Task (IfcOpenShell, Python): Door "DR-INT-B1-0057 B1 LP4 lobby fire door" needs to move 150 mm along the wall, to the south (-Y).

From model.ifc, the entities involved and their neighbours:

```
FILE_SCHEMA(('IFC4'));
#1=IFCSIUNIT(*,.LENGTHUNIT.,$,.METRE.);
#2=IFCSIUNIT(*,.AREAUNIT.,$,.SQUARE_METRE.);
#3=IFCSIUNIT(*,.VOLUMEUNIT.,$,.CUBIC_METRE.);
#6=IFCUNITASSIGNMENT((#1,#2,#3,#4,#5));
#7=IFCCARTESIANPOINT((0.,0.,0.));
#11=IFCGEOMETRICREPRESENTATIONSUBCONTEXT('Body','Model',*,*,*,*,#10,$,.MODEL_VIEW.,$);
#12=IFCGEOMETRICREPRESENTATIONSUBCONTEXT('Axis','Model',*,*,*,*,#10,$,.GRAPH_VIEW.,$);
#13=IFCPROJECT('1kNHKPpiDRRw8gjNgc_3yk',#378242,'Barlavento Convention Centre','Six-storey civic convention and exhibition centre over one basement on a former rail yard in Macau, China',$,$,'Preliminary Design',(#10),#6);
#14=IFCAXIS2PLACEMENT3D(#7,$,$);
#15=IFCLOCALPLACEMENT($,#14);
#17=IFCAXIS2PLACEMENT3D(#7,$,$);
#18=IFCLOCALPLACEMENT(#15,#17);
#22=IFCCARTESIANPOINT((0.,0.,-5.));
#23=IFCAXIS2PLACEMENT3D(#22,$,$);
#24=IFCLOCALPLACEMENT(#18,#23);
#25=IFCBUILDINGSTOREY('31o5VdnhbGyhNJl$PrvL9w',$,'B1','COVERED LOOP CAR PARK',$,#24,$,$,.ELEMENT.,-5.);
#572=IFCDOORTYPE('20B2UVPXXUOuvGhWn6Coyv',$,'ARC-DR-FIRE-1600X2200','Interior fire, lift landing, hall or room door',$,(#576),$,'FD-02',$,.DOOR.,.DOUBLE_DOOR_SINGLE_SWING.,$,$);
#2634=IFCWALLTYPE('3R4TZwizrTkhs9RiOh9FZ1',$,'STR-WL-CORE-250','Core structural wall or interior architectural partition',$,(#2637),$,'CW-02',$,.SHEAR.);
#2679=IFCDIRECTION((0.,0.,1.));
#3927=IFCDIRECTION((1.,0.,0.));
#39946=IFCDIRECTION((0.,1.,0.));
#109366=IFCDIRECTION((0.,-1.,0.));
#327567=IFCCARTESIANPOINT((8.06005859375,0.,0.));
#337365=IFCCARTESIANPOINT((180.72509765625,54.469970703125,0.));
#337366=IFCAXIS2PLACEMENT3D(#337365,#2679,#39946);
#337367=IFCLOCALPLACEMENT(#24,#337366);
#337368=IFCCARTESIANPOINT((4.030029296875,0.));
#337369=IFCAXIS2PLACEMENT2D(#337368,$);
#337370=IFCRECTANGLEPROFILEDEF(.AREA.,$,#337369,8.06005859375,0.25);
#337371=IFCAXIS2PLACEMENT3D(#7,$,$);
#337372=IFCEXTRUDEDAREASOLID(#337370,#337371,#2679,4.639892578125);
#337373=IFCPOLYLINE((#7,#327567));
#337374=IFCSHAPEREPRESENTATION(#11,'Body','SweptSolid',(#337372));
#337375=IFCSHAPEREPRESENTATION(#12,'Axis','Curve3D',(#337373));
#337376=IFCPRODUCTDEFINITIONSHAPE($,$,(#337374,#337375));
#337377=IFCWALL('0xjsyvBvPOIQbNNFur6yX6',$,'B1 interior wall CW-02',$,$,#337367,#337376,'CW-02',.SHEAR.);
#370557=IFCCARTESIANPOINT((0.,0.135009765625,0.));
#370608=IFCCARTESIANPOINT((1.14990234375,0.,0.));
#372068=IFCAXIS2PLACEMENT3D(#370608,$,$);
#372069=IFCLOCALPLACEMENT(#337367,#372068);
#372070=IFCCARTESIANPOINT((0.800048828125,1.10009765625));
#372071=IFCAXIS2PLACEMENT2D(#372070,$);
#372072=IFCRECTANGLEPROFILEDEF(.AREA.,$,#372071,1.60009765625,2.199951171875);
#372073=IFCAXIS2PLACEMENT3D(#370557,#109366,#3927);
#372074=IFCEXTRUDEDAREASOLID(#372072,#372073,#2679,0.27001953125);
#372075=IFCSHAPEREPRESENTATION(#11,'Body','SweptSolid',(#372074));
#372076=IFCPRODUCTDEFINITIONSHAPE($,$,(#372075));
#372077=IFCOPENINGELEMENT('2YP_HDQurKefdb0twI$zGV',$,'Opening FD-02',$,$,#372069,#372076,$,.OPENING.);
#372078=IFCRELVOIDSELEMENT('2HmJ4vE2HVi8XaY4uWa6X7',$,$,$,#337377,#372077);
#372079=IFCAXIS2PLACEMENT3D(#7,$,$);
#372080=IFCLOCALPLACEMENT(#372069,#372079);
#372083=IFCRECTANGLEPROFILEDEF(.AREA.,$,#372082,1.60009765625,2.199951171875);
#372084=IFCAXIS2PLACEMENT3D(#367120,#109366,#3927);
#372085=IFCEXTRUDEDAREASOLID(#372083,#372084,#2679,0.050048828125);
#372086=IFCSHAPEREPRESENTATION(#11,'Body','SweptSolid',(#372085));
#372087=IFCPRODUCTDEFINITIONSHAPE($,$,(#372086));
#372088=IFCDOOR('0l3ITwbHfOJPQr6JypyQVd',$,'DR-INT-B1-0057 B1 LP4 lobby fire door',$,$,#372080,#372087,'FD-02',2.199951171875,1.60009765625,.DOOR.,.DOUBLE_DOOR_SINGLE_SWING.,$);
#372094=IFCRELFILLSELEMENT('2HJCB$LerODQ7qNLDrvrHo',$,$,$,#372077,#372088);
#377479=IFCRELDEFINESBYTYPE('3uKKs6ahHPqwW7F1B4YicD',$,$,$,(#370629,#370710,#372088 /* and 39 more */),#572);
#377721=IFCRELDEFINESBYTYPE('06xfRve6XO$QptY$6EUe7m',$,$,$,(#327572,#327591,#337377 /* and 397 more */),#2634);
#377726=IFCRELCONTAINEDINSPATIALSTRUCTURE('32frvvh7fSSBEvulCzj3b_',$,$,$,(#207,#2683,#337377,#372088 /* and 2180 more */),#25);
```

```python
import ifcopenshell
import ifcopenshell.api.geometry
import ifcopenshell.util.placement

model = ifcopenshell.open("model.ifc")

door = model.by_guid("0l3ITwbHfOJPQr6JypyQVd")
opening = door.FillsVoids[0].RelatingOpeningElement
wall = opening.VoidsElements[0].RelatingBuildingElement

wall_matrix = ifcopenshell.util.placement.get_local_placement(wall.ObjectPlacement)
shift = wall_matrix[:3, 0] * -0.15
before = ifcopenshell.util.placement.get_local_placement(door.ObjectPlacement)[:3, 3].copy()

# The door is placed relative to its opening, so it follows when the opening moves.
matrix = ifcopenshell.util.placement.get_local_placement(opening.ObjectPlacement)
matrix[:3, 3] += shift
ifcopenshell.api.geometry.edit_object_placement(
    model, product=opening, matrix=matrix, is_si=False, should_transform_children=True
)

after = ifcopenshell.util.placement.get_local_placement(door.ObjectPlacement)[:3, 3]
print("door moved by", (after - before).round(3) + 0.0)

model.write("model_v2.ifc")
```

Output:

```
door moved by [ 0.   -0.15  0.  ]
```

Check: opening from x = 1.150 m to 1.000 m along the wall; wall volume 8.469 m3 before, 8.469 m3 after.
